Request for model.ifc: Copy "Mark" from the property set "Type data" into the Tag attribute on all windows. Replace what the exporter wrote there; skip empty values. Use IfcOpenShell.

First a look at what the model holds.

```python
import ifcopenshell
import ifcopenshell.util.element

model = ifcopenshell.open("model.ifc")
print(model.schema)
windows = model.by_type("IfcWindow")
print(len(windows), "windows")
for e in windows[:8]:
    source = ifcopenshell.util.element.get_pset(e, "Type data", "Mark")
    target = e.Tag
    print(e.id(), repr(source), repr(target), sep=" | ")
```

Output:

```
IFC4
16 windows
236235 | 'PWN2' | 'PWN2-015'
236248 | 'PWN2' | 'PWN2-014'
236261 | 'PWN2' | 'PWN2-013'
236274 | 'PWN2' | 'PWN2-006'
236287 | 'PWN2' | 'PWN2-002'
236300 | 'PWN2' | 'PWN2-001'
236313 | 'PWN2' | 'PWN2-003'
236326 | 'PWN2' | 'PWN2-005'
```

```python
import ifcopenshell
import ifcopenshell.util.element

model = ifcopenshell.open("model.ifc")

count = 0
for e in model.by_type("IfcWindow"):
    value = ifcopenshell.util.element.get_pset(e, "Type data", "Mark")
    current = e.Tag
    if not value or not value.strip() or current == value:
        continue
    e.Tag = value
    count += 1

print(count, "windows updated")

model.write("model-out.ifc")
```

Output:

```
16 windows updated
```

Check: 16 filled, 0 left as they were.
